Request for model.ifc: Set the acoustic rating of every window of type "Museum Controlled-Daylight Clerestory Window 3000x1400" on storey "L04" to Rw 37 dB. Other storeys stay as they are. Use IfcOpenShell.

First a look at what the model holds.

```python
import ifcopenshell
import ifcopenshell.util.element

model = ifcopenshell.open("model.ifc")
print(model.schema)
storey = next(s for s in model.by_type("IfcBuildingStorey") if s.Name == "L04")
windows = [e for e in ifcopenshell.util.element.get_decomposition(storey) if e.is_a("IfcWindow")]
seen = {}
for e in windows:
    element_type = ifcopenshell.util.element.get_type(e)
    key = (element_type.Name if element_type != e and element_type else None, ifcopenshell.util.element.get_pset(e, "Pset_WindowCommon", "AcousticRating"))
    seen[key] = seen.get(key, 0) + 1
for (name, value), count in sorted(seen.items(), key=str):
    print(count, "x", name, "|", value)
```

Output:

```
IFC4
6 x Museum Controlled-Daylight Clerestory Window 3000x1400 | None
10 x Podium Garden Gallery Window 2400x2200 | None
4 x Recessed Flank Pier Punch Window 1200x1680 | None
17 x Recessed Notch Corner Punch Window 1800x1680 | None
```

```python
import ifcopenshell
import ifcopenshell.api.pset
import ifcopenshell.util.element

model = ifcopenshell.open("model.ifc")

storey = next(s for s in model.by_type("IfcBuildingStorey") if s.Name == "L04")
windows = [e for e in ifcopenshell.util.element.get_decomposition(storey) if e.is_a("IfcWindow")]

count = 0
for e in windows:
    element_type = ifcopenshell.util.element.get_type(e)
    if element_type in (None, e) or element_type.Name != "Museum Controlled-Daylight Clerestory Window 3000x1400":
        continue
    found = ifcopenshell.util.element.get_pset(e, "Pset_WindowCommon", should_inherit=False)
    if found:
        pset = model.by_id(found["id"])
        if len(ifcopenshell.util.element.get_elements_by_pset(pset)) > 1:
            pset = ifcopenshell.api.pset.unshare_pset(model, products=[e], pset=pset)[0]
    else:
        pset = ifcopenshell.api.pset.add_pset(model, product=e, name="Pset_WindowCommon")
    ifcopenshell.api.pset.edit_pset(model, pset=pset, properties={"AcousticRating": "Rw 37 dB"})
    count += 1

print(count, "windows updated")

model.write("model_rev.ifc")
```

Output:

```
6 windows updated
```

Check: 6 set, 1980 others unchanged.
